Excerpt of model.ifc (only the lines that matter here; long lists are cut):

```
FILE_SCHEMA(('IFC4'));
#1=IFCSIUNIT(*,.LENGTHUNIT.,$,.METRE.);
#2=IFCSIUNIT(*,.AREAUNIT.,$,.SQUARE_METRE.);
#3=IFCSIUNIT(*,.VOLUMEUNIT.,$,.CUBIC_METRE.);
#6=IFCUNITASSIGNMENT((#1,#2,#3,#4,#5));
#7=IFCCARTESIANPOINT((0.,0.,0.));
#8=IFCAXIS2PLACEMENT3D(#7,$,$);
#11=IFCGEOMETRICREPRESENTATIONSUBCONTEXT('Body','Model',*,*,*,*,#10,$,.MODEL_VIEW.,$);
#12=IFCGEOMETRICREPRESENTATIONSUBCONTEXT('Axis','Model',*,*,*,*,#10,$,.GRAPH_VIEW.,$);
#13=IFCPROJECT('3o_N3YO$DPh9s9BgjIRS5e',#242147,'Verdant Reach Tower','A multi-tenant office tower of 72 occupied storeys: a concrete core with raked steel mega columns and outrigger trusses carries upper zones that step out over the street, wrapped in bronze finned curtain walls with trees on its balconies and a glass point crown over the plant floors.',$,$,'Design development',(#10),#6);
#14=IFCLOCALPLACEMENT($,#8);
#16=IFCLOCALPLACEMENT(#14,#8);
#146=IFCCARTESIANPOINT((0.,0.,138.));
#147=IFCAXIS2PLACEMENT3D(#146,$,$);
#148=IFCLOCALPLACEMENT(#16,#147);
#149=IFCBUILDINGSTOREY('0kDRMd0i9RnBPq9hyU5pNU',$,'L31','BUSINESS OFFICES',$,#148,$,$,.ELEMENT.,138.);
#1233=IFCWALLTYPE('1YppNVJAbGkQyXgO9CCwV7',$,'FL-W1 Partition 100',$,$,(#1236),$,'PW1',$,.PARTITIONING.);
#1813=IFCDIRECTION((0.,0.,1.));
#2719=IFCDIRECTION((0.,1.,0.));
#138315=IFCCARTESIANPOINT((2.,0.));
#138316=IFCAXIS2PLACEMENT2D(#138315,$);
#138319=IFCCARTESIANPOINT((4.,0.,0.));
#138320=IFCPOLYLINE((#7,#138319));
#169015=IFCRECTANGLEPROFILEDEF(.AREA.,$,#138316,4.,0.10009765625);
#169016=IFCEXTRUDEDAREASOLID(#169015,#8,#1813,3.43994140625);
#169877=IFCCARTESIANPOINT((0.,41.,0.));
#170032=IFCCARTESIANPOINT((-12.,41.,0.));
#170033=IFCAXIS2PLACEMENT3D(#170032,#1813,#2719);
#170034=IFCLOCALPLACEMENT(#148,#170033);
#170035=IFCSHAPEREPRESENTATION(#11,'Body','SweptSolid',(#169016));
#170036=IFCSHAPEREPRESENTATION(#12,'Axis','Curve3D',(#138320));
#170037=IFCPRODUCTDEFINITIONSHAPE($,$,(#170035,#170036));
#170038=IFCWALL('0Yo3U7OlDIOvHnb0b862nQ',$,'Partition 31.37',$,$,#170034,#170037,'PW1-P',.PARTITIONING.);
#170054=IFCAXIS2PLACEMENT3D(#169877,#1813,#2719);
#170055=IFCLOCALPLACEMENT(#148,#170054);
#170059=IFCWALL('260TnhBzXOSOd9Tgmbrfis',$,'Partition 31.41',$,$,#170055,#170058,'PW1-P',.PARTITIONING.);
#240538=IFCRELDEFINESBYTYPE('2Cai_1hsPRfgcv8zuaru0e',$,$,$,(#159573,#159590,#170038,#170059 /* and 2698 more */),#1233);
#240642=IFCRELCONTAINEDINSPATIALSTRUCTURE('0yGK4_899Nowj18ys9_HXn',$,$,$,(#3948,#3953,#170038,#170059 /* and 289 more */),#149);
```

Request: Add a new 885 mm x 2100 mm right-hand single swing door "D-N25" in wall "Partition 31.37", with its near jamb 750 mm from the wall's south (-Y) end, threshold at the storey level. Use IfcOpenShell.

```python
import numpy as np
import ifcopenshell
import ifcopenshell.api.feature
import ifcopenshell.api.geometry
import ifcopenshell.api.root
import ifcopenshell.api.spatial
import ifcopenshell.geom
import ifcopenshell.util.element
import ifcopenshell.util.placement
import ifcopenshell.util.representation
import ifcopenshell.util.shape
import ifcopenshell.util.unit

model = ifcopenshell.open("model.ifc")
unit_scale = ifcopenshell.util.unit.calculate_unit_scale(model)
settings = ifcopenshell.geom.settings()


def volume(element):
    """Net volume in cubic metres, openings subtracted."""
    shape = ifcopenshell.geom.create_shape(settings, element)
    return ifcopenshell.util.shape.get_volume(shape.geometry)


wall = model.by_id(170038)
storey = ifcopenshell.util.element.get_container(wall, ifc_class="IfcBuildingStorey")
context = ifcopenshell.util.representation.get_context(model, "Model", "Body", "MODEL_VIEW")
before = volume(wall)

width, height, from_end, sill = 0.885, 2.1, 0.75, 0.0  # metres

# The wall runs along its own X axis, and the end named is its -X end.
wall_shape = ifcopenshell.geom.create_shape(settings, wall)
x, y, z = ifcopenshell.util.shape.get_vertices(wall_shape.geometry).T
start = x.min() + from_end
face, thickness = float(y.min()), float(y.max() - y.min())
wall_matrix = ifcopenshell.util.placement.get_local_placement(wall.ObjectPlacement)
level = ifcopenshell.util.placement.get_local_placement(storey.ObjectPlacement)[2, 3]


def in_wall(x, y):
    """Placement at x, y metres in the wall's axes, at sill height."""
    matrix = wall_matrix.copy()
    matrix[:, 3] = wall_matrix @ np.array([x / unit_scale, y / unit_scale, 0.0, 1.0])
    matrix[2, 3] = level + sill / unit_scale
    return matrix


# Opening: a box that overshoots both wall faces by 50 mm.
opening = ifcopenshell.api.root.create_entity(model, ifc_class="IfcOpeningElement", predefined_type="OPENING")
box = ifcopenshell.api.geometry.add_wall_representation(
    model, context=context, length=width, height=height, thickness=thickness + 0.1
)
ifcopenshell.api.geometry.assign_representation(model, product=opening, representation=box)
ifcopenshell.api.geometry.edit_object_placement(model, product=opening, matrix=in_wall(start, face - 0.05), is_si=False)
ifcopenshell.api.feature.add_feature(model, feature=opening, element=wall)

door = ifcopenshell.api.root.create_entity(model, ifc_class="IfcDoor", name="D-N25", predefined_type="DOOR")
door.OverallWidth, door.OverallHeight = width / unit_scale, height / unit_scale
door.OperationType = "SINGLE_SWING_RIGHT"
body = ifcopenshell.api.geometry.add_door_representation(
    model,
    context=context,
    overall_width=door.OverallWidth,
    overall_height=door.OverallHeight,
    operation_type="SINGLE_SWING_RIGHT",
    lining_properties={"LiningDepth": thickness / unit_scale, "ThresholdDepth": thickness / unit_scale},
)
ifcopenshell.api.geometry.assign_representation(model, product=door, representation=body)
ifcopenshell.api.spatial.assign_container(model, products=[door], relating_structure=storey)
ifcopenshell.api.feature.add_filling(model, opening=opening, element=door)

# The lining spans the wall, so the door starts at the wall face.
ifcopenshell.api.geometry.edit_object_placement(model, product=door, matrix=in_wall(start, face), is_si=False)

after = volume(wall)

print(f"wall volume {before:.3f} -> {after:.3f} m3")

model.write("model-out.ifc")
```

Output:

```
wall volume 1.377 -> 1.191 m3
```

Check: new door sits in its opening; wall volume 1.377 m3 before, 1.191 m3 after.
